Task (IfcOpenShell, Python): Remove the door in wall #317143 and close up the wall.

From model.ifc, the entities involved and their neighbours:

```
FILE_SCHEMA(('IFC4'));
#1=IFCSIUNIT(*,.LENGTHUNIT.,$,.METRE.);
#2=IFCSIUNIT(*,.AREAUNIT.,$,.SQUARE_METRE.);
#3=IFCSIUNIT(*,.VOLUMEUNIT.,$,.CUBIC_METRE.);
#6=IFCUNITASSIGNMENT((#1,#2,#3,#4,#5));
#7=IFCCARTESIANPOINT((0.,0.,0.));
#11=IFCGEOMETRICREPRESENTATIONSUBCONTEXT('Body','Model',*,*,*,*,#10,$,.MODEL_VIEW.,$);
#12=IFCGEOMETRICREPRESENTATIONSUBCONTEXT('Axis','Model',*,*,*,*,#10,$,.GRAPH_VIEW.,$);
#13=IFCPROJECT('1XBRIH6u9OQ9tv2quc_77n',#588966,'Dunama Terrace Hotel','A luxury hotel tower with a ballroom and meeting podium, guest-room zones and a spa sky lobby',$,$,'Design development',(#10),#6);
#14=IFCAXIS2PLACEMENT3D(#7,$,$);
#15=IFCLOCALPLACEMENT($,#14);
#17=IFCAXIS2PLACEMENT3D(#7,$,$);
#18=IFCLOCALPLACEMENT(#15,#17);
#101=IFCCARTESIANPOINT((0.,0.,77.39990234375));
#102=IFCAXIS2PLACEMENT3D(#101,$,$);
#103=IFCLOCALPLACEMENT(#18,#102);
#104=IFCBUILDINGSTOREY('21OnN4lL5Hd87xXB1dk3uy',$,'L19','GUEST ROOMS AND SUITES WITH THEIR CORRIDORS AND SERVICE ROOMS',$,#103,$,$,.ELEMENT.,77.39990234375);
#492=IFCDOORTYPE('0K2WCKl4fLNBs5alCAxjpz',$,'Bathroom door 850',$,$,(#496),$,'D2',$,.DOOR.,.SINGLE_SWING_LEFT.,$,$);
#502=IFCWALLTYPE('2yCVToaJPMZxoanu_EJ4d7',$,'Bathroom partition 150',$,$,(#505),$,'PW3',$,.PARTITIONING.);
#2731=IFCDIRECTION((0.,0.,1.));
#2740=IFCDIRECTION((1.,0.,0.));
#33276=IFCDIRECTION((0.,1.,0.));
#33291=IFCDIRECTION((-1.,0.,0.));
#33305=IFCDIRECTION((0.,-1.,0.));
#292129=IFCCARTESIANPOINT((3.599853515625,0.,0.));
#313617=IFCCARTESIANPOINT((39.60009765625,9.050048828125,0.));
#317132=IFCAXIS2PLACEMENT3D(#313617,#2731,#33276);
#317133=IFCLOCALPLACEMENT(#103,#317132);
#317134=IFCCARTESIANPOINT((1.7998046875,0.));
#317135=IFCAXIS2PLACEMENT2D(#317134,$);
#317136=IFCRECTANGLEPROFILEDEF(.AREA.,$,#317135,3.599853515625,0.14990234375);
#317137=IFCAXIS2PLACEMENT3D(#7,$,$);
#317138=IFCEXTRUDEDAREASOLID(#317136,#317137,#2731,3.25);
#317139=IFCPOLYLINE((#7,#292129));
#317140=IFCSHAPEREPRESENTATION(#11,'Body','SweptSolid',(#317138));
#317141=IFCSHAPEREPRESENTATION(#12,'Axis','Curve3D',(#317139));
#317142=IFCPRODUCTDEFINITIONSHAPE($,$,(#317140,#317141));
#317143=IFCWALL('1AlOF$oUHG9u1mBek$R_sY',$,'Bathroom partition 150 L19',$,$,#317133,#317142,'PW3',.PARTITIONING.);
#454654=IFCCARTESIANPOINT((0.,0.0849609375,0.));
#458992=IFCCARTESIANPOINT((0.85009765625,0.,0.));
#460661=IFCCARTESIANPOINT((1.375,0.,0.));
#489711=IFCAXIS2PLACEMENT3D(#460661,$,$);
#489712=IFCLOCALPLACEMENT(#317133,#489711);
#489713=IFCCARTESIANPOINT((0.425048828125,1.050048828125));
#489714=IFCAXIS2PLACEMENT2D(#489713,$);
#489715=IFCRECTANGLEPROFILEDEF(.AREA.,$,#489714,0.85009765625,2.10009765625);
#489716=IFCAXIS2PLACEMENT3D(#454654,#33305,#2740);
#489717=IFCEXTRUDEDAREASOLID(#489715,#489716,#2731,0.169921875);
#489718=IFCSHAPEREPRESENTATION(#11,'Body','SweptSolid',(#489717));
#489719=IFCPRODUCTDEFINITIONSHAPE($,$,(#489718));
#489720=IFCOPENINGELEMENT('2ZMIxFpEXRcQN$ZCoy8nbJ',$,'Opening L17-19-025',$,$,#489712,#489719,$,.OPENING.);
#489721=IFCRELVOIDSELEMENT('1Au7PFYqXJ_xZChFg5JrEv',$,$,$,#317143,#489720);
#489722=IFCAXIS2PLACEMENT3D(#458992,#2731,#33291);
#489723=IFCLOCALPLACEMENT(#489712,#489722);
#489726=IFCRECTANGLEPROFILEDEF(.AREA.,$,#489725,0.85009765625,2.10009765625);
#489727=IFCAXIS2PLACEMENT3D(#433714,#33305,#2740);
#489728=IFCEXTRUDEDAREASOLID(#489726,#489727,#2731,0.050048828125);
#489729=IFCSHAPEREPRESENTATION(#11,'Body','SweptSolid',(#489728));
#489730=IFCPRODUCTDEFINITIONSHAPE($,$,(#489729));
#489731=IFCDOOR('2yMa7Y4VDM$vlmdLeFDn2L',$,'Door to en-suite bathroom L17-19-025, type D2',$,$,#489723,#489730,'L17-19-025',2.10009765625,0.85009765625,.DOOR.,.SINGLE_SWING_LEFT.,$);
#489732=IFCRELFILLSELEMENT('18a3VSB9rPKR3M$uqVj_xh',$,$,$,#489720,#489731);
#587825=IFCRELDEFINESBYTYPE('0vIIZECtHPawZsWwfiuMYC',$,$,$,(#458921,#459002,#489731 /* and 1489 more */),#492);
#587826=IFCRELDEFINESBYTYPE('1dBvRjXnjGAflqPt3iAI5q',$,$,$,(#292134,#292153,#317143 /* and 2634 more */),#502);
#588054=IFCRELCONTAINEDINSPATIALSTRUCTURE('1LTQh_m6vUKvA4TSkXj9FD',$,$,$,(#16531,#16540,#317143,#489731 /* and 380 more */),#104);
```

```python
import ifcopenshell
import ifcopenshell.api.feature
import ifcopenshell.api.root
import ifcopenshell.geom
import ifcopenshell.util.shape

model = ifcopenshell.open("model.ifc")
settings = ifcopenshell.geom.settings()


def volume(element):
    """Net volume in cubic metres, openings subtracted."""
    shape = ifcopenshell.geom.create_shape(settings, element)
    return ifcopenshell.util.shape.get_volume(shape.geometry)


door = model.by_guid("2yMa7Y4VDM$vlmdLeFDn2L")
opening = door.FillsVoids[0].RelatingOpeningElement
wall = opening.VoidsElements[0].RelatingBuildingElement
before = volume(wall)

ifcopenshell.api.root.remove_product(model, product=door)
ifcopenshell.api.feature.remove_feature(model, feature=opening)

after = volume(wall)

print(f"wall volume {before:.3f} -> {after:.3f} m3")

model.write("model_rev.ifc")
```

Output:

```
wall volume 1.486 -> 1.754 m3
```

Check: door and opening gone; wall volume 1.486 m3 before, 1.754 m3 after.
